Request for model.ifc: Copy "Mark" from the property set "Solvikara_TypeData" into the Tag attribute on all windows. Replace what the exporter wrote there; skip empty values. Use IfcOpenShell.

First a look at what the model holds.

```python
import ifcopenshell
import ifcopenshell.util.element

model = ifcopenshell.open("model.ifc")
print(model.schema)
windows = model.by_type("IfcWindow")
print(len(windows), "windows")
for e in windows[:8]:
    source = ifcopenshell.util.element.get_pset(e, "Solvikara_TypeData", "Mark")
    target = e.Tag
    print(e.id(), repr(source), repr(target), sep=" | ")
```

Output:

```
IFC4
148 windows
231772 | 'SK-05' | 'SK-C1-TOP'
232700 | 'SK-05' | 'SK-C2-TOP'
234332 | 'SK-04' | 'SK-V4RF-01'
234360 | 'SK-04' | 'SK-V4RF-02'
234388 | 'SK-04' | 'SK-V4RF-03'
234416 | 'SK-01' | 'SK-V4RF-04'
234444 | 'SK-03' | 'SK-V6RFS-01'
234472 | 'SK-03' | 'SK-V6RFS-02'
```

```python
import ifcopenshell
import ifcopenshell.util.element

model = ifcopenshell.open("model.ifc")

count = 0
for e in model.by_type("IfcWindow"):
    value = ifcopenshell.util.element.get_pset(e, "Solvikara_TypeData", "Mark")
    current = e.Tag
    if not value or not value.strip() or current == value:
        continue
    e.Tag = value
    count += 1

print(count, "windows updated")

model.write("model-out.ifc")
```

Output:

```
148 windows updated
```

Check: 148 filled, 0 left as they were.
